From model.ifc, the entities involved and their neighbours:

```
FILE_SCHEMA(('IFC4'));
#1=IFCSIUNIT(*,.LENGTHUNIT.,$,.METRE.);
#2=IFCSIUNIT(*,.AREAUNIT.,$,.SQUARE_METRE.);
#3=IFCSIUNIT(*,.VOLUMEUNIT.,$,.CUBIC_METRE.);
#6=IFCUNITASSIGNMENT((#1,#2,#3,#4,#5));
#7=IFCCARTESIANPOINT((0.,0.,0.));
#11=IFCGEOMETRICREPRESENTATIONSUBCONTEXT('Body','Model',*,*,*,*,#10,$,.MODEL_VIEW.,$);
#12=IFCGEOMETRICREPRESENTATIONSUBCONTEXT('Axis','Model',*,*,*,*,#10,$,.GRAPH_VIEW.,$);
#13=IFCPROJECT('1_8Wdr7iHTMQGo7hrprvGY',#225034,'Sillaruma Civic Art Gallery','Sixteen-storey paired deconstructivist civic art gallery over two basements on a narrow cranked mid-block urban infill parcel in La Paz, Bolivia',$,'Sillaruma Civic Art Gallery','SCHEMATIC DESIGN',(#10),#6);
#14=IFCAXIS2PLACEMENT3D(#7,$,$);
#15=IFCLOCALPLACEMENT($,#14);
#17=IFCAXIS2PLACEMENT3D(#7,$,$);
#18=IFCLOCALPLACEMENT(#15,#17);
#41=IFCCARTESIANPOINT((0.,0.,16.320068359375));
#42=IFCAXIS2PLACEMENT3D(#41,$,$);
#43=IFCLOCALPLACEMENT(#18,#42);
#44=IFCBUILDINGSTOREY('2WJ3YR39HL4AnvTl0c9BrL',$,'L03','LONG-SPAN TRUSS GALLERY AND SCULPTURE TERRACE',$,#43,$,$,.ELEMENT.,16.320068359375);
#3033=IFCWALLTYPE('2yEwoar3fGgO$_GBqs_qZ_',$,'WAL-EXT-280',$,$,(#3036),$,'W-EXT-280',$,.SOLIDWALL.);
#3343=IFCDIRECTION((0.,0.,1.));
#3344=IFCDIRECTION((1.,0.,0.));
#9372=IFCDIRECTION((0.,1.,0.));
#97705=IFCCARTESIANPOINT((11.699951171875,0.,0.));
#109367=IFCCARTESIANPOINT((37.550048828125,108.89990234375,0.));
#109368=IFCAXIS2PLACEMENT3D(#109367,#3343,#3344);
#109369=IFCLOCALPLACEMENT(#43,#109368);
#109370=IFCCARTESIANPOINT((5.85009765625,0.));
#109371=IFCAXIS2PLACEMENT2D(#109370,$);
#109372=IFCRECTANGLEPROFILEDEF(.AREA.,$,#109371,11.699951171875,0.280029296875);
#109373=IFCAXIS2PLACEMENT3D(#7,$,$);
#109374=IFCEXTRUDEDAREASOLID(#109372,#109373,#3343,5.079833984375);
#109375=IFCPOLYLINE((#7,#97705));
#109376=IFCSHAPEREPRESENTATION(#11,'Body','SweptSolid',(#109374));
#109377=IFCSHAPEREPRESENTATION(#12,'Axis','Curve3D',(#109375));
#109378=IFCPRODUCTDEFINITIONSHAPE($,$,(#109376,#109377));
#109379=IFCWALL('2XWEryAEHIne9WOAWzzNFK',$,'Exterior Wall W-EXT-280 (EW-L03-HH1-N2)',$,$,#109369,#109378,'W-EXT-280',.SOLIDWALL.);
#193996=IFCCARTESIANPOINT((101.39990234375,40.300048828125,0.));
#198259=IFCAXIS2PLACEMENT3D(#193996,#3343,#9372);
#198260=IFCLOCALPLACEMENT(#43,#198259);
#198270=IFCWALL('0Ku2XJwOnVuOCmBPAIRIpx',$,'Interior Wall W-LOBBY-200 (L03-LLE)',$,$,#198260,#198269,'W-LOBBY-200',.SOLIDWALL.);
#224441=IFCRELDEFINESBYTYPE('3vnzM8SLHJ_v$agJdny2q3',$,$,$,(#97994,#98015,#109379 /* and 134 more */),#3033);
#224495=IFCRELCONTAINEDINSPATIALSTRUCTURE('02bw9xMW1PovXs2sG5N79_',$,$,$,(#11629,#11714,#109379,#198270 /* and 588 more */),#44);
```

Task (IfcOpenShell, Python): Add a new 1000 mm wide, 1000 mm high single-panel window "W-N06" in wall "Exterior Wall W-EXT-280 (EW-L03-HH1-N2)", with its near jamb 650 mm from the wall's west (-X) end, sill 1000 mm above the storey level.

```python
import numpy as np
import ifcopenshell
import ifcopenshell.api.feature
import ifcopenshell.api.geometry
import ifcopenshell.api.root
import ifcopenshell.api.spatial
import ifcopenshell.geom
import ifcopenshell.util.element
import ifcopenshell.util.placement
import ifcopenshell.util.representation
import ifcopenshell.util.shape
import ifcopenshell.util.unit

model = ifcopenshell.open("model.ifc")
unit_scale = ifcopenshell.util.unit.calculate_unit_scale(model)
settings = ifcopenshell.geom.settings()


def volume(element):
    """Net volume in cubic metres, openings subtracted."""
    shape = ifcopenshell.geom.create_shape(settings, element)
    return ifcopenshell.util.shape.get_volume(shape.geometry)


wall = model.by_id(109379)
storey = ifcopenshell.util.element.get_container(wall, ifc_class="IfcBuildingStorey")
context = ifcopenshell.util.representation.get_context(model, "Model", "Body", "MODEL_VIEW")
before = volume(wall)

width, height, from_end, sill = 1, 1, 0.65, 1  # metres

# The wall runs along its own X axis, and the end named is its -X end.
wall_shape = ifcopenshell.geom.create_shape(settings, wall)
x, y, z = ifcopenshell.util.shape.get_vertices(wall_shape.geometry).T
start = x.min() + from_end
face, thickness = float(y.min()), float(y.max() - y.min())
wall_matrix = ifcopenshell.util.placement.get_local_placement(wall.ObjectPlacement)
level = ifcopenshell.util.placement.get_local_placement(storey.ObjectPlacement)[2, 3]


def in_wall(x, y):
    """Placement at x, y metres in the wall's axes, at sill height."""
    matrix = wall_matrix.copy()
    matrix[:, 3] = wall_matrix @ np.array([x / unit_scale, y / unit_scale, 0.0, 1.0])
    matrix[2, 3] = level + sill / unit_scale
    return matrix


# Opening: a box that overshoots both wall faces by 50 mm.
opening = ifcopenshell.api.root.create_entity(model, ifc_class="IfcOpeningElement", predefined_type="OPENING")
box = ifcopenshell.api.geometry.add_wall_representation(
    model, context=context, length=width, height=height, thickness=thickness + 0.1
)
ifcopenshell.api.geometry.assign_representation(model, product=opening, representation=box)
ifcopenshell.api.geometry.edit_object_placement(model, product=opening, matrix=in_wall(start, face - 0.05), is_si=False)
ifcopenshell.api.feature.add_feature(model, feature=opening, element=wall)

window = ifcopenshell.api.root.create_entity(model, ifc_class="IfcWindow", name="W-N06", predefined_type="WINDOW")
window.OverallWidth, window.OverallHeight = width / unit_scale, height / unit_scale
window.PartitioningType = "SINGLE_PANEL"
body = ifcopenshell.api.geometry.add_window_representation(
    model,
    context=context,
    overall_width=window.OverallWidth,
    overall_height=window.OverallHeight,
    partition_type="SINGLE_PANEL",
)
ifcopenshell.api.geometry.assign_representation(model, product=window, representation=body)
ifcopenshell.api.spatial.assign_container(model, products=[window], relating_structure=storey)
ifcopenshell.api.feature.add_filling(model, opening=opening, element=window)

# Centre the window in the wall's thickness.
ifcopenshell.api.geometry.edit_object_placement(model, product=window, matrix=in_wall(start, face), is_si=False)
window_shape = ifcopenshell.geom.create_shape(settings, window)
depth = ifcopenshell.util.shape.get_vertices(window_shape.geometry)[:, 1]
offset = face + thickness / 2 - (depth.min() + depth.max()) / 2
ifcopenshell.api.geometry.edit_object_placement(model, product=window, matrix=in_wall(start, offset), is_si=False)

after = volume(wall)

print(f"wall volume {before:.3f} -> {after:.3f} m3")

model.write("model_updated.ifc")
```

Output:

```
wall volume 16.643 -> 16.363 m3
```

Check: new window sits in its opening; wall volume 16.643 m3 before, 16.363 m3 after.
